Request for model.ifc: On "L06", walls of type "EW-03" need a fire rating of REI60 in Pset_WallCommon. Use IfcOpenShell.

First a look at what the model holds.

```python
import ifcopenshell
import ifcopenshell.util.element

model = ifcopenshell.open("model.ifc")
print(model.schema)
storey = next(s for s in model.by_type("IfcBuildingStorey") if s.Name == "L06")
walls = [e for e in ifcopenshell.util.element.get_decomposition(storey) if e.is_a("IfcWall")]
seen = {}
for e in walls:
    element_type = ifcopenshell.util.element.get_type(e)
    key = (element_type.Name if element_type != e and element_type else None, ifcopenshell.util.element.get_pset(e, "Pset_WallCommon", "FireRating"))
    seen[key] = seen.get(key, 0) + 1
for (name, value), count in sorted(seen.items(), key=str):
    print(count, "x", name, "|", value)
```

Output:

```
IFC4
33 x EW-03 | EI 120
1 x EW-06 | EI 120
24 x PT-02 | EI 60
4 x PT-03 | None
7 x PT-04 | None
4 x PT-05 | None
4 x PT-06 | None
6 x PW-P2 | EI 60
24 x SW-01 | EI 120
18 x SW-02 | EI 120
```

```python
import ifcopenshell
import ifcopenshell.api.pset
import ifcopenshell.util.element

model = ifcopenshell.open("model.ifc")

storey = next(s for s in model.by_type("IfcBuildingStorey") if s.Name == "L06")
walls = [e for e in ifcopenshell.util.element.get_decomposition(storey) if e.is_a("IfcWall")]

count = 0
for e in walls:
    element_type = ifcopenshell.util.element.get_type(e)
    if element_type in (None, e) or element_type.Name != "EW-03":
        continue
    # add_pset returns the element's existing set when there is one.
    pset = ifcopenshell.api.pset.add_pset(model, product=e, name="Pset_WallCommon")
    ifcopenshell.api.pset.edit_pset(model, pset=pset, properties={"FireRating": "REI60"})
    count += 1

print(count, "walls updated")

model.write("model-out.ifc")
```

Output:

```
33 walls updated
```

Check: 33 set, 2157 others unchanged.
